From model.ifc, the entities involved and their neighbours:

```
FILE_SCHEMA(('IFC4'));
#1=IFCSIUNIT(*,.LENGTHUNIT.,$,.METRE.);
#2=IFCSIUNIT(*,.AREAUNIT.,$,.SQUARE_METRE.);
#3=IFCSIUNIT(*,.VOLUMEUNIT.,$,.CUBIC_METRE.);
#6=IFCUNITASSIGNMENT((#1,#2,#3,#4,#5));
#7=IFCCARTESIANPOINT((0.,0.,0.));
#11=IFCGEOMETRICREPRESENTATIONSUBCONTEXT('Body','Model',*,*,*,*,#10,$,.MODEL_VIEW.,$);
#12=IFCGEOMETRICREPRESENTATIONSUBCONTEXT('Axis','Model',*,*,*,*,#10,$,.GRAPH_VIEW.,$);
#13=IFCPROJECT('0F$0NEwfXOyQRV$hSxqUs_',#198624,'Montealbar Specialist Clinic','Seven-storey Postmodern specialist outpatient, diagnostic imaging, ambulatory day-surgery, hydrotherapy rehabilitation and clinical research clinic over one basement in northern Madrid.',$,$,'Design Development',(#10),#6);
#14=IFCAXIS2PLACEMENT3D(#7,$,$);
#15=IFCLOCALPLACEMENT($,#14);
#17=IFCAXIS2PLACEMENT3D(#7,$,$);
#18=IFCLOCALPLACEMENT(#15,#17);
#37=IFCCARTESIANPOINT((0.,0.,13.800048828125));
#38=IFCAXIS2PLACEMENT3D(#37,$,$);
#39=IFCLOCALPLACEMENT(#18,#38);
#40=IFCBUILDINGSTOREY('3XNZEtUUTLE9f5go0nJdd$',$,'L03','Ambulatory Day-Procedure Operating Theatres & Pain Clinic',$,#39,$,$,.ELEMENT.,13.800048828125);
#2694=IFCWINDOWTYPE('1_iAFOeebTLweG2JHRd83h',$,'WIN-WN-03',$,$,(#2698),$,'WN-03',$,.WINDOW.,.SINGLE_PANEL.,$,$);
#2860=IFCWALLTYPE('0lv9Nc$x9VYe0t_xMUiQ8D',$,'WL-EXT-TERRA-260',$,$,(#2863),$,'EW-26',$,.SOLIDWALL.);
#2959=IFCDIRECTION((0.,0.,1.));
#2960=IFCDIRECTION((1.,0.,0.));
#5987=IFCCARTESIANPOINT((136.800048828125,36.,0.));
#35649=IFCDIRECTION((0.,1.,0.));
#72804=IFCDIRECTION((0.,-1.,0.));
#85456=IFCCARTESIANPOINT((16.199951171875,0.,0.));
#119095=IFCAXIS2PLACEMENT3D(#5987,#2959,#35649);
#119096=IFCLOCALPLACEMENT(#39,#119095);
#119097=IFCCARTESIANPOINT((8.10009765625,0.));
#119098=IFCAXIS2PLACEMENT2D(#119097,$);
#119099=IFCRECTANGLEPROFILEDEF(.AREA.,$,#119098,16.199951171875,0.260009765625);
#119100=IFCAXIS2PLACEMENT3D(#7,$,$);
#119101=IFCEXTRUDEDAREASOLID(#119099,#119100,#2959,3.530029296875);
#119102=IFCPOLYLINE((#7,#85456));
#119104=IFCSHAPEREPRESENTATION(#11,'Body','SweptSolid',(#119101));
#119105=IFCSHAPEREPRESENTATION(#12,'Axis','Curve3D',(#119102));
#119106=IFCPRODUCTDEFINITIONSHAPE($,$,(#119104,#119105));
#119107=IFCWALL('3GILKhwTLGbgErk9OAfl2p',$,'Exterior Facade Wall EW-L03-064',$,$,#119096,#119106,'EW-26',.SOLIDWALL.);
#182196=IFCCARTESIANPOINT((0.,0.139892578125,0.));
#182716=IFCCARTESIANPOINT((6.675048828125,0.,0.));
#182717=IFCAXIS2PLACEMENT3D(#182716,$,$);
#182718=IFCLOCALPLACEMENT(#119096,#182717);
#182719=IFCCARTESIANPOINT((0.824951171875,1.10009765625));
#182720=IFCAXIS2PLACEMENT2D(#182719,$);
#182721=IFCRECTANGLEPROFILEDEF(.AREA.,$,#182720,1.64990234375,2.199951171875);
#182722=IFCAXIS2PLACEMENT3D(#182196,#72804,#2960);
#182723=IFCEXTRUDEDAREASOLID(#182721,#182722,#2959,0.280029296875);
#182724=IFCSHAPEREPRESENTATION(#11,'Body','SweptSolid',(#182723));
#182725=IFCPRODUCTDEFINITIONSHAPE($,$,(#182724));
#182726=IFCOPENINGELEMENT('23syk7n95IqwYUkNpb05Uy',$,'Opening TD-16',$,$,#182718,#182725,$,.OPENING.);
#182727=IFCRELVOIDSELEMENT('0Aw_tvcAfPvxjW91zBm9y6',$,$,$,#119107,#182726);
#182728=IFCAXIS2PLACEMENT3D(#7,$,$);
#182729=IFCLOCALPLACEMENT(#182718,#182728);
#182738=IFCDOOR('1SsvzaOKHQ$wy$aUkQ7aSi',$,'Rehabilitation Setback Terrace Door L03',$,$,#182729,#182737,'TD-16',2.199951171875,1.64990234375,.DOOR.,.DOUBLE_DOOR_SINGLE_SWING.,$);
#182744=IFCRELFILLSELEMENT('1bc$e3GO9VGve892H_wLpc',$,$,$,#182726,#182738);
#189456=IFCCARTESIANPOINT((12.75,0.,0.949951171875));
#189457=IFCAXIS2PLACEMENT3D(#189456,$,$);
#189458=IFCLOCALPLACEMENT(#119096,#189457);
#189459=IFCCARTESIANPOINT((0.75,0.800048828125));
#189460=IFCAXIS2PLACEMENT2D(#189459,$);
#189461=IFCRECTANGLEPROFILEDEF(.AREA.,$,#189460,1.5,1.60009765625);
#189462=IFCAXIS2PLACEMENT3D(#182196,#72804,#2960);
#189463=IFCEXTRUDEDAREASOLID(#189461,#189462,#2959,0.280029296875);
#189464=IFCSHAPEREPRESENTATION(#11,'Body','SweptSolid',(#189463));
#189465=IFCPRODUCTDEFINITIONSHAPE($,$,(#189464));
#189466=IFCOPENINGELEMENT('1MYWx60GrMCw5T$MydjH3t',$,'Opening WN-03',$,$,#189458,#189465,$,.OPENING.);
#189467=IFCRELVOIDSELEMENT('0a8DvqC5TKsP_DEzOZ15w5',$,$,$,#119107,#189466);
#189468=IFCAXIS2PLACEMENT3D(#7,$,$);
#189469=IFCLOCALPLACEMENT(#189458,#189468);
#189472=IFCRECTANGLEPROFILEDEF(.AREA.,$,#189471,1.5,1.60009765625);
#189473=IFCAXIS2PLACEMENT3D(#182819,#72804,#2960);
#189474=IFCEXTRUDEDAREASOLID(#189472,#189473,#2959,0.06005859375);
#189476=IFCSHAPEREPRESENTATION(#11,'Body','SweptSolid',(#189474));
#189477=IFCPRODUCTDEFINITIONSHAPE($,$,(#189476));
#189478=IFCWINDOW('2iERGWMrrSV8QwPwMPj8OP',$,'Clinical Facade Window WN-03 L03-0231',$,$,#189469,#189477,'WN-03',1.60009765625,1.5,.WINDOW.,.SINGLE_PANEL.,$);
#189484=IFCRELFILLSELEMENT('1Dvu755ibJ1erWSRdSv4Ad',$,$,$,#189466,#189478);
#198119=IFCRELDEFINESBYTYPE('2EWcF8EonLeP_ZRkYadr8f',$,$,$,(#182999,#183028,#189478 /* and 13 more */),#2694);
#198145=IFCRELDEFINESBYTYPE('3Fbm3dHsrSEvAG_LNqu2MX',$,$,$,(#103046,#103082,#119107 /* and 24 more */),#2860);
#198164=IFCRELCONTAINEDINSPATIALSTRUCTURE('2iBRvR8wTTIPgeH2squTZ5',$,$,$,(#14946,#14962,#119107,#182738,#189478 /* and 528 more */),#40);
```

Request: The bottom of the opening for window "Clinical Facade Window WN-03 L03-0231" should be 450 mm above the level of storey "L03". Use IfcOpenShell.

```python
import numpy as np
import ifcopenshell
import ifcopenshell.api.geometry
import ifcopenshell.geom
import ifcopenshell.util.element
import ifcopenshell.util.placement
import ifcopenshell.util.shape
import ifcopenshell.util.unit

model = ifcopenshell.open("model.ifc")
unit_scale = ifcopenshell.util.unit.calculate_unit_scale(model)

window = model.by_guid("2iERGWMrrSV8QwPwMPj8OP")
opening = window.FillsVoids[0].RelatingOpeningElement
storey = ifcopenshell.util.element.get_container(window, ifc_class="IfcBuildingStorey")
level = ifcopenshell.util.placement.get_local_placement(storey.ObjectPlacement)[2, 3]

# The opening's origin need not be at the sill, so measure its lowest point.
shape = ifcopenshell.geom.create_shape(ifcopenshell.geom.settings(), opening)
bottom = ifcopenshell.util.shape.get_shape_bottom_elevation(shape, shape.geometry) / unit_scale
dz = level + 0.45 - bottom

shift = np.array([0.0, 0.0, dz])
# The window is placed relative to its opening, so it follows when the opening moves.
matrix = ifcopenshell.util.placement.get_local_placement(opening.ObjectPlacement)
matrix[:3, 3] += shift
ifcopenshell.api.geometry.edit_object_placement(
    model, product=opening, matrix=matrix, is_si=False, should_transform_children=True
)

print(f"moved by {dz * unit_scale:+.3f} m")

model.write("model_updated.ifc")
```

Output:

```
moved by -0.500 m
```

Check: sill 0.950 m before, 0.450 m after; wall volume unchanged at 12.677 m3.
